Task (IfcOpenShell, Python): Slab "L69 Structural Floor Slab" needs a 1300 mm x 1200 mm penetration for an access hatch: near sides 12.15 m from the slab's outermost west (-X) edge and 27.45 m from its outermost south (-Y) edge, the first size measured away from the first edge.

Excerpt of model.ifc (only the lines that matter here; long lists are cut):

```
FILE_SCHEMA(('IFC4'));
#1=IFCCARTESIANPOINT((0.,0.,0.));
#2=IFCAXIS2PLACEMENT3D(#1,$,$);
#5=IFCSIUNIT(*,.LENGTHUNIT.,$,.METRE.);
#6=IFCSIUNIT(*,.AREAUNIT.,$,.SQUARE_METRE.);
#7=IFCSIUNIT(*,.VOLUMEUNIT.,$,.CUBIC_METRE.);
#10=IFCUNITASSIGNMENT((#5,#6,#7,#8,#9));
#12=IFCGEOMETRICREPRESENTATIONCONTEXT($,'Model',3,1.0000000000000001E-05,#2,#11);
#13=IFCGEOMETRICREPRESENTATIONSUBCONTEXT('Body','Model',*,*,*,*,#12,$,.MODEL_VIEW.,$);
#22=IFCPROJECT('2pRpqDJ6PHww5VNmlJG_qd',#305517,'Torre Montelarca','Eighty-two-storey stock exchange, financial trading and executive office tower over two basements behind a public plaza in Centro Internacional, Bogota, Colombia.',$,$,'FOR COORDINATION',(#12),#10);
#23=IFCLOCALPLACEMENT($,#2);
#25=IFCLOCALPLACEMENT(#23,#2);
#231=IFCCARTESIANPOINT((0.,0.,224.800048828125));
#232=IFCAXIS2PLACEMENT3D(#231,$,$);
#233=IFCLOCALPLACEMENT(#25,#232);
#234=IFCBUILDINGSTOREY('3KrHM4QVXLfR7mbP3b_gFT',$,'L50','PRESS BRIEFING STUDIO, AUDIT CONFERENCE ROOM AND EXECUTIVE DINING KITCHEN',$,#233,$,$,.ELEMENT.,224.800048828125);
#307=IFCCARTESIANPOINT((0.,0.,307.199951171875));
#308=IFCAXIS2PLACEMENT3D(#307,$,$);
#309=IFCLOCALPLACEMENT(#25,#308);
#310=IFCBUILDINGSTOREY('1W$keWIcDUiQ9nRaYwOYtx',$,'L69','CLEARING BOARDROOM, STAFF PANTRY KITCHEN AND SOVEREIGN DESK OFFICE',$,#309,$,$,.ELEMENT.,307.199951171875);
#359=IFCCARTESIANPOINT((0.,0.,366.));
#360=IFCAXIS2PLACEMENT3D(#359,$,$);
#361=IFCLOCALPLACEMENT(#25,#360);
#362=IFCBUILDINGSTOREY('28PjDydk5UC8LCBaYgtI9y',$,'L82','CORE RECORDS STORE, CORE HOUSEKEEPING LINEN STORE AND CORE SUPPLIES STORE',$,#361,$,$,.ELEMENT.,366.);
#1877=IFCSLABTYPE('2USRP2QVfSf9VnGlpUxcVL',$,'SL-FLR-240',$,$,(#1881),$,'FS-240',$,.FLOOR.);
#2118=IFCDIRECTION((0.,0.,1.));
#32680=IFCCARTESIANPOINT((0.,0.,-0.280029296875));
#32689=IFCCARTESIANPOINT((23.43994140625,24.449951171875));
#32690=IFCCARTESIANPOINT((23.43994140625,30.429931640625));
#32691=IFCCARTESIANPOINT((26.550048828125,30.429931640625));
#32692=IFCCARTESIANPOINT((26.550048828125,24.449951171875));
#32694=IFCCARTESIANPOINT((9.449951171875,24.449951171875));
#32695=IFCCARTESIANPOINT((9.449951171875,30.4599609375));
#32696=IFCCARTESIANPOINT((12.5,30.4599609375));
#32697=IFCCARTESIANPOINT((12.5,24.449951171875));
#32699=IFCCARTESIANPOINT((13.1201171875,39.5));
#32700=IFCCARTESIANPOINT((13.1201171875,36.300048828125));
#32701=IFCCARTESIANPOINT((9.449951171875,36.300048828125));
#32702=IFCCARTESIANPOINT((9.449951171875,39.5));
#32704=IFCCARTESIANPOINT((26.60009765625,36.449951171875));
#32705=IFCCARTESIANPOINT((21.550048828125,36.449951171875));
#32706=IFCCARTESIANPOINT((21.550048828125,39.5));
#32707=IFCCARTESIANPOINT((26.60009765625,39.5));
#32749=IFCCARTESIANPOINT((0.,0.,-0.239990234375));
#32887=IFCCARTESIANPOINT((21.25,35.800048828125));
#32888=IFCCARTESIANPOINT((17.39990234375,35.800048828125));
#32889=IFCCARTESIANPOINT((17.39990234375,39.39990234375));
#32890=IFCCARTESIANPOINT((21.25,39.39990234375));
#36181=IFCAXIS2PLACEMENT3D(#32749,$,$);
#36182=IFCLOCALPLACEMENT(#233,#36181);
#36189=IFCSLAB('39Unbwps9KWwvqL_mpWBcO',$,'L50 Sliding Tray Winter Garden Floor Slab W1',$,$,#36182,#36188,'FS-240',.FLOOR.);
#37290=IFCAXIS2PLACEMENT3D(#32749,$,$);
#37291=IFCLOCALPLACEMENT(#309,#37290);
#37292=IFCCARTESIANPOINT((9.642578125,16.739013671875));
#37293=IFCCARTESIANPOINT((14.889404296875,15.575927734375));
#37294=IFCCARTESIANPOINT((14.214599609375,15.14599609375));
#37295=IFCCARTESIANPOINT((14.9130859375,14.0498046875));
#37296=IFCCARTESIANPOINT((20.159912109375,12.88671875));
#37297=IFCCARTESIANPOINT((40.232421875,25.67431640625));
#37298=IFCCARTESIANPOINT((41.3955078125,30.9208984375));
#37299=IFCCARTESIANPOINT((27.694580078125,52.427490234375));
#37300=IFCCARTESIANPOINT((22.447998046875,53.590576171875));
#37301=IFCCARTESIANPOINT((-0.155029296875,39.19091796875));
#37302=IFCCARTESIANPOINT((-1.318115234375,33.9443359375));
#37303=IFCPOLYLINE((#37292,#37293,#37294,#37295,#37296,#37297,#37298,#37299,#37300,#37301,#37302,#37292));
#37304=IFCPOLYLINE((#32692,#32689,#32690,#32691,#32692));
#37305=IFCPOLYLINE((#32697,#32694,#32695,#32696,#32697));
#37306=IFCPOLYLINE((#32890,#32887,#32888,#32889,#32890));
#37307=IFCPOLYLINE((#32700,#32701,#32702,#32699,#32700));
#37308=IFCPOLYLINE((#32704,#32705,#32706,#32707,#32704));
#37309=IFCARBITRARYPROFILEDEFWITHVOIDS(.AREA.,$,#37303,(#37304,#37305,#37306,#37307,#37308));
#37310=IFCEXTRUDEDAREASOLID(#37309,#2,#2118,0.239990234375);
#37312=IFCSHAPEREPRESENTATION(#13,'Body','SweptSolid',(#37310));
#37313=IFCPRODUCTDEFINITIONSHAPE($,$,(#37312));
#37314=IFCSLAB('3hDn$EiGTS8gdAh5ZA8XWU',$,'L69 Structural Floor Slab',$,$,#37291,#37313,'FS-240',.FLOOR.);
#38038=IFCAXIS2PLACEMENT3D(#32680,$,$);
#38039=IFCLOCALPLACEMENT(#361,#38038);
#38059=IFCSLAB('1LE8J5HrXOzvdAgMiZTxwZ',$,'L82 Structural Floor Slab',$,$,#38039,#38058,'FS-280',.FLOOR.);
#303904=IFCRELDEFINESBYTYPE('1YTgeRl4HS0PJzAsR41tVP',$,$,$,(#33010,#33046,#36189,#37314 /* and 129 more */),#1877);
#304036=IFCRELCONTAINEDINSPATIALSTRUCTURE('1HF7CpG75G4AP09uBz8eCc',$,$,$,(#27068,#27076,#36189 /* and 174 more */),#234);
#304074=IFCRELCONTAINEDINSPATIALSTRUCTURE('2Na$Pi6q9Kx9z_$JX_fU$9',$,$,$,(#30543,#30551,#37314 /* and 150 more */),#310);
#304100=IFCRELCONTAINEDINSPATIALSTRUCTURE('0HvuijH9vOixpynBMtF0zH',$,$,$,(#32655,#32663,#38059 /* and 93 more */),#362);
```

```python
import numpy as np
import ifcopenshell
import ifcopenshell.api.feature
import ifcopenshell.api.geometry
import ifcopenshell.api.root
import ifcopenshell.geom
import ifcopenshell.util.placement
import ifcopenshell.util.representation
import ifcopenshell.util.shape
import ifcopenshell.util.unit

model = ifcopenshell.open("model.ifc")
unit_scale = ifcopenshell.util.unit.calculate_unit_scale(model)
settings = ifcopenshell.geom.settings()


def volume(element):
    """Net volume in cubic metres, openings subtracted."""
    shape = ifcopenshell.geom.create_shape(settings, element)
    return ifcopenshell.util.shape.get_volume(shape.geometry)


slab = model.by_guid("3hDn$EiGTS8gdAh5ZA8XWU")
before = volume(slab)

# Extent in the slab's own axes, in metres. The edges named are its -X and -Y sides.
slab_shape = ifcopenshell.geom.create_shape(settings, slab)
vertices = ifcopenshell.util.shape.get_vertices(slab_shape.geometry)
x_min, y_min, bottom = vertices.min(axis=0)
top = vertices[:, 2].max()

opening = ifcopenshell.api.root.create_entity(model, ifc_class="IfcOpeningElement", name="Access hatch opening", predefined_type="OPENING")
context = ifcopenshell.util.representation.get_context(model, "Model", "Body", "MODEL_VIEW")
width, depth = 1.3, 1.2
outline = [(0.0, 0.0), (width, 0.0), (width, depth), (0.0, depth), (0.0, 0.0)]
# Overshoot both faces by 50 mm so the cut is clean.
shape = ifcopenshell.api.geometry.add_slab_representation(
    model, context=context, depth=top - bottom + 0.1, polyline=outline
)
ifcopenshell.api.geometry.assign_representation(model, product=opening, representation=shape)

matrix = ifcopenshell.util.placement.get_local_placement(slab.ObjectPlacement)
matrix[:, 3] = matrix @ np.append(np.array([x_min + 12.15, y_min + 27.45, bottom - 0.05]) / unit_scale, 1.0)
ifcopenshell.api.geometry.edit_object_placement(model, product=opening, matrix=matrix, is_si=False)
ifcopenshell.api.feature.add_feature(model, feature=opening, element=slab)

after = volume(slab)

print(f"slab volume {before:.3f} -> {after:.3f} m3")

model.write("model_updated.ifc")
```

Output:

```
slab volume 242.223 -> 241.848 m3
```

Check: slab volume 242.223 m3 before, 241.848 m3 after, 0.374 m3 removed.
